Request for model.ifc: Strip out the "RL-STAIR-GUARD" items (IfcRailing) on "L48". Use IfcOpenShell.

First a look at what the model holds.

```python
import ifcopenshell
import ifcopenshell.util.element

model = ifcopenshell.open("model.ifc")
print(model.schema)
storey = next(s for s in model.by_type("IfcBuildingStorey") if s.Name == "L48")
railings = [e for e in ifcopenshell.util.element.get_decomposition(storey) if e.is_a("IfcRailing")]
seen = {}
for e in railings:
    element_type = ifcopenshell.util.element.get_type(e)
    name = element_type.Name if element_type not in (None, e) else None
    seen[name] = seen.get(name, 0) + 1
for name, count in sorted(seen.items(), key=str):
    print(count, "x", name)
```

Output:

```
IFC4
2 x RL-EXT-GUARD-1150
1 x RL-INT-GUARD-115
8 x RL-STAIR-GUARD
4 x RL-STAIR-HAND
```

```python
import ifcopenshell
import ifcopenshell.api.root
import ifcopenshell.util.element

model = ifcopenshell.open("model.ifc")

storey = next(s for s in model.by_type("IfcBuildingStorey") if s.Name == "L48")
railings = [e for e in ifcopenshell.util.element.get_decomposition(storey) if e.is_a("IfcRailing")]
targets = [e for e in railings if (t := ifcopenshell.util.element.get_type(e)) not in (None, e) and t.Name == "RL-STAIR-GUARD"]

for e in targets:
    ifcopenshell.api.root.remove_product(model, product=e)
print(len(targets), "removed")

model.write("model_edited.ifc")
```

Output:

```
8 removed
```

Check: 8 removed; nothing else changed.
